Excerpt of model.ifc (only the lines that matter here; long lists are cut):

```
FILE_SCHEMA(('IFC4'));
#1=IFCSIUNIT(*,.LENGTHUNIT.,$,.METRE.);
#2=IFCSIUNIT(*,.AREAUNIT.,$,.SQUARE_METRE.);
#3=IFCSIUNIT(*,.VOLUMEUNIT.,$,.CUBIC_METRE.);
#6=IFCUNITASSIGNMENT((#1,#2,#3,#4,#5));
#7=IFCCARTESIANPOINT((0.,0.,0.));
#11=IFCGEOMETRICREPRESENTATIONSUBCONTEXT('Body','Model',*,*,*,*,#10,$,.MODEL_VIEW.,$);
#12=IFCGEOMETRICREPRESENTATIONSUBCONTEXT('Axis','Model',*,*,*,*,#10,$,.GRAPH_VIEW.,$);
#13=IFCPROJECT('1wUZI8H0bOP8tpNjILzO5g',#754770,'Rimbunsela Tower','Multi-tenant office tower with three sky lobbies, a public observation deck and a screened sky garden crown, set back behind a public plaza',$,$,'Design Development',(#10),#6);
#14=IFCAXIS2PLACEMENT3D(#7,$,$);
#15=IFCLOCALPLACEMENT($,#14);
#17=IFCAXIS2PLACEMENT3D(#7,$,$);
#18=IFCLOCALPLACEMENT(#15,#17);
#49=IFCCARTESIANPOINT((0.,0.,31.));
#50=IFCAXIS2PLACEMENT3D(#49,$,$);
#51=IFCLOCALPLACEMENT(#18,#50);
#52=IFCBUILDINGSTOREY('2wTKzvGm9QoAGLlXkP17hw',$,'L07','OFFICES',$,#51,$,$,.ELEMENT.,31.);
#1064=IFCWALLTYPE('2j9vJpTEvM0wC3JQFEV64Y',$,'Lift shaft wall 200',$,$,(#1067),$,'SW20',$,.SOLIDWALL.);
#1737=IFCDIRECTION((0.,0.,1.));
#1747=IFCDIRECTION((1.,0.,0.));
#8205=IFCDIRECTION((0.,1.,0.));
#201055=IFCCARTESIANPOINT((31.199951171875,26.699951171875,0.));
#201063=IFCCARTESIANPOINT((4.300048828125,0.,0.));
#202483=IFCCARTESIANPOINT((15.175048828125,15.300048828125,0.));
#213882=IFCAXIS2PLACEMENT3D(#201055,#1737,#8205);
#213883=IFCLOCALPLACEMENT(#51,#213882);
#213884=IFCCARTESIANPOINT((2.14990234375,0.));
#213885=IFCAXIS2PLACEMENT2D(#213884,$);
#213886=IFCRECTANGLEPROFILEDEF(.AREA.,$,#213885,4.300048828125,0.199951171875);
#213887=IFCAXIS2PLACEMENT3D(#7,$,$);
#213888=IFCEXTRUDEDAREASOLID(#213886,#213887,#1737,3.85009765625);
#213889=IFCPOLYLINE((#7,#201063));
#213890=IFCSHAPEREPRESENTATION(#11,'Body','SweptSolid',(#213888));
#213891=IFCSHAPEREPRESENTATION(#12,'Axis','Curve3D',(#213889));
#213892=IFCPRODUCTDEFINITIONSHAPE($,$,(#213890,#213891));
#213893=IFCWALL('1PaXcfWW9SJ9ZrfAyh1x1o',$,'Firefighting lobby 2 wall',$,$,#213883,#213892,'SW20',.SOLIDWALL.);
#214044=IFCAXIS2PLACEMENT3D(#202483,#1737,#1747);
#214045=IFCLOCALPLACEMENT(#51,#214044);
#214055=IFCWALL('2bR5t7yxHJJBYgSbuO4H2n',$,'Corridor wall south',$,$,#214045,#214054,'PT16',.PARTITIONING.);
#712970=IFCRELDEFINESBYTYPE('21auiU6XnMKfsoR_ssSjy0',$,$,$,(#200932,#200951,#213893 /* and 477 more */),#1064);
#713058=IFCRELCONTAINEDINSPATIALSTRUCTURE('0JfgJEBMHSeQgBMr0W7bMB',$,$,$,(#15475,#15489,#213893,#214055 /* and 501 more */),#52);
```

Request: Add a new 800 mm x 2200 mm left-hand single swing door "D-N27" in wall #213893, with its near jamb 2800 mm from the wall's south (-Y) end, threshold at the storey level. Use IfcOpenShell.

```python
import numpy as np
import ifcopenshell
import ifcopenshell.api.feature
import ifcopenshell.api.geometry
import ifcopenshell.api.root
import ifcopenshell.api.spatial
import ifcopenshell.geom
import ifcopenshell.util.element
import ifcopenshell.util.placement
import ifcopenshell.util.representation
import ifcopenshell.util.shape
import ifcopenshell.util.unit

model = ifcopenshell.open("model.ifc")
unit_scale = ifcopenshell.util.unit.calculate_unit_scale(model)
settings = ifcopenshell.geom.settings()


def volume(element):
    """Net volume in cubic metres, openings subtracted."""
    shape = ifcopenshell.geom.create_shape(settings, element)
    return ifcopenshell.util.shape.get_volume(shape.geometry)


wall = model.by_guid("1PaXcfWW9SJ9ZrfAyh1x1o")
storey = ifcopenshell.util.element.get_container(wall, ifc_class="IfcBuildingStorey")
context = ifcopenshell.util.representation.get_context(model, "Model", "Body", "MODEL_VIEW")
before = volume(wall)

width, height, from_end, sill = 0.8, 2.2, 2.8, 0.0  # metres

# The wall runs along its own X axis, and the end named is its -X end.
wall_shape = ifcopenshell.geom.create_shape(settings, wall)
x, y, z = ifcopenshell.util.shape.get_vertices(wall_shape.geometry).T
start = x.min() + from_end
face, thickness = float(y.min()), float(y.max() - y.min())
wall_matrix = ifcopenshell.util.placement.get_local_placement(wall.ObjectPlacement)
level = ifcopenshell.util.placement.get_local_placement(storey.ObjectPlacement)[2, 3]


def in_wall(x, y):
    """Placement at x, y metres in the wall's axes, at sill height."""
    matrix = wall_matrix.copy()
    matrix[:, 3] = wall_matrix @ np.array([x / unit_scale, y / unit_scale, 0.0, 1.0])
    matrix[2, 3] = level + sill / unit_scale
    return matrix


# Opening: a box that overshoots both wall faces by 50 mm.
opening = ifcopenshell.api.root.create_entity(model, ifc_class="IfcOpeningElement", predefined_type="OPENING")
box = ifcopenshell.api.geometry.add_wall_representation(
    model, context=context, length=width, height=height, thickness=thickness + 0.1
)
ifcopenshell.api.geometry.assign_representation(model, product=opening, representation=box)
ifcopenshell.api.geometry.edit_object_placement(model, product=opening, matrix=in_wall(start, face - 0.05), is_si=False)
ifcopenshell.api.feature.add_feature(model, feature=opening, element=wall)

door = ifcopenshell.api.root.create_entity(model, ifc_class="IfcDoor", name="D-N27", predefined_type="DOOR")
door.OverallWidth, door.OverallHeight = width / unit_scale, height / unit_scale
door.OperationType = "SINGLE_SWING_LEFT"
body = ifcopenshell.api.geometry.add_door_representation(
    model,
    context=context,
    overall_width=door.OverallWidth,
    overall_height=door.OverallHeight,
    operation_type="SINGLE_SWING_LEFT",
    lining_properties={"LiningDepth": thickness / unit_scale, "ThresholdDepth": thickness / unit_scale},
)
ifcopenshell.api.geometry.assign_representation(model, product=door, representation=body)
ifcopenshell.api.spatial.assign_container(model, products=[door], relating_structure=storey)
ifcopenshell.api.feature.add_filling(model, opening=opening, element=door)

# The lining spans the wall, so the door starts at the wall face.
ifcopenshell.api.geometry.edit_object_placement(model, product=door, matrix=in_wall(start, face), is_si=False)

after = volume(wall)

print(f"wall volume {before:.3f} -> {after:.3f} m3")

model.write("model_v2.ifc")
```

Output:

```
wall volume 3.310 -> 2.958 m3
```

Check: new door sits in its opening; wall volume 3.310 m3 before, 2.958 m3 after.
